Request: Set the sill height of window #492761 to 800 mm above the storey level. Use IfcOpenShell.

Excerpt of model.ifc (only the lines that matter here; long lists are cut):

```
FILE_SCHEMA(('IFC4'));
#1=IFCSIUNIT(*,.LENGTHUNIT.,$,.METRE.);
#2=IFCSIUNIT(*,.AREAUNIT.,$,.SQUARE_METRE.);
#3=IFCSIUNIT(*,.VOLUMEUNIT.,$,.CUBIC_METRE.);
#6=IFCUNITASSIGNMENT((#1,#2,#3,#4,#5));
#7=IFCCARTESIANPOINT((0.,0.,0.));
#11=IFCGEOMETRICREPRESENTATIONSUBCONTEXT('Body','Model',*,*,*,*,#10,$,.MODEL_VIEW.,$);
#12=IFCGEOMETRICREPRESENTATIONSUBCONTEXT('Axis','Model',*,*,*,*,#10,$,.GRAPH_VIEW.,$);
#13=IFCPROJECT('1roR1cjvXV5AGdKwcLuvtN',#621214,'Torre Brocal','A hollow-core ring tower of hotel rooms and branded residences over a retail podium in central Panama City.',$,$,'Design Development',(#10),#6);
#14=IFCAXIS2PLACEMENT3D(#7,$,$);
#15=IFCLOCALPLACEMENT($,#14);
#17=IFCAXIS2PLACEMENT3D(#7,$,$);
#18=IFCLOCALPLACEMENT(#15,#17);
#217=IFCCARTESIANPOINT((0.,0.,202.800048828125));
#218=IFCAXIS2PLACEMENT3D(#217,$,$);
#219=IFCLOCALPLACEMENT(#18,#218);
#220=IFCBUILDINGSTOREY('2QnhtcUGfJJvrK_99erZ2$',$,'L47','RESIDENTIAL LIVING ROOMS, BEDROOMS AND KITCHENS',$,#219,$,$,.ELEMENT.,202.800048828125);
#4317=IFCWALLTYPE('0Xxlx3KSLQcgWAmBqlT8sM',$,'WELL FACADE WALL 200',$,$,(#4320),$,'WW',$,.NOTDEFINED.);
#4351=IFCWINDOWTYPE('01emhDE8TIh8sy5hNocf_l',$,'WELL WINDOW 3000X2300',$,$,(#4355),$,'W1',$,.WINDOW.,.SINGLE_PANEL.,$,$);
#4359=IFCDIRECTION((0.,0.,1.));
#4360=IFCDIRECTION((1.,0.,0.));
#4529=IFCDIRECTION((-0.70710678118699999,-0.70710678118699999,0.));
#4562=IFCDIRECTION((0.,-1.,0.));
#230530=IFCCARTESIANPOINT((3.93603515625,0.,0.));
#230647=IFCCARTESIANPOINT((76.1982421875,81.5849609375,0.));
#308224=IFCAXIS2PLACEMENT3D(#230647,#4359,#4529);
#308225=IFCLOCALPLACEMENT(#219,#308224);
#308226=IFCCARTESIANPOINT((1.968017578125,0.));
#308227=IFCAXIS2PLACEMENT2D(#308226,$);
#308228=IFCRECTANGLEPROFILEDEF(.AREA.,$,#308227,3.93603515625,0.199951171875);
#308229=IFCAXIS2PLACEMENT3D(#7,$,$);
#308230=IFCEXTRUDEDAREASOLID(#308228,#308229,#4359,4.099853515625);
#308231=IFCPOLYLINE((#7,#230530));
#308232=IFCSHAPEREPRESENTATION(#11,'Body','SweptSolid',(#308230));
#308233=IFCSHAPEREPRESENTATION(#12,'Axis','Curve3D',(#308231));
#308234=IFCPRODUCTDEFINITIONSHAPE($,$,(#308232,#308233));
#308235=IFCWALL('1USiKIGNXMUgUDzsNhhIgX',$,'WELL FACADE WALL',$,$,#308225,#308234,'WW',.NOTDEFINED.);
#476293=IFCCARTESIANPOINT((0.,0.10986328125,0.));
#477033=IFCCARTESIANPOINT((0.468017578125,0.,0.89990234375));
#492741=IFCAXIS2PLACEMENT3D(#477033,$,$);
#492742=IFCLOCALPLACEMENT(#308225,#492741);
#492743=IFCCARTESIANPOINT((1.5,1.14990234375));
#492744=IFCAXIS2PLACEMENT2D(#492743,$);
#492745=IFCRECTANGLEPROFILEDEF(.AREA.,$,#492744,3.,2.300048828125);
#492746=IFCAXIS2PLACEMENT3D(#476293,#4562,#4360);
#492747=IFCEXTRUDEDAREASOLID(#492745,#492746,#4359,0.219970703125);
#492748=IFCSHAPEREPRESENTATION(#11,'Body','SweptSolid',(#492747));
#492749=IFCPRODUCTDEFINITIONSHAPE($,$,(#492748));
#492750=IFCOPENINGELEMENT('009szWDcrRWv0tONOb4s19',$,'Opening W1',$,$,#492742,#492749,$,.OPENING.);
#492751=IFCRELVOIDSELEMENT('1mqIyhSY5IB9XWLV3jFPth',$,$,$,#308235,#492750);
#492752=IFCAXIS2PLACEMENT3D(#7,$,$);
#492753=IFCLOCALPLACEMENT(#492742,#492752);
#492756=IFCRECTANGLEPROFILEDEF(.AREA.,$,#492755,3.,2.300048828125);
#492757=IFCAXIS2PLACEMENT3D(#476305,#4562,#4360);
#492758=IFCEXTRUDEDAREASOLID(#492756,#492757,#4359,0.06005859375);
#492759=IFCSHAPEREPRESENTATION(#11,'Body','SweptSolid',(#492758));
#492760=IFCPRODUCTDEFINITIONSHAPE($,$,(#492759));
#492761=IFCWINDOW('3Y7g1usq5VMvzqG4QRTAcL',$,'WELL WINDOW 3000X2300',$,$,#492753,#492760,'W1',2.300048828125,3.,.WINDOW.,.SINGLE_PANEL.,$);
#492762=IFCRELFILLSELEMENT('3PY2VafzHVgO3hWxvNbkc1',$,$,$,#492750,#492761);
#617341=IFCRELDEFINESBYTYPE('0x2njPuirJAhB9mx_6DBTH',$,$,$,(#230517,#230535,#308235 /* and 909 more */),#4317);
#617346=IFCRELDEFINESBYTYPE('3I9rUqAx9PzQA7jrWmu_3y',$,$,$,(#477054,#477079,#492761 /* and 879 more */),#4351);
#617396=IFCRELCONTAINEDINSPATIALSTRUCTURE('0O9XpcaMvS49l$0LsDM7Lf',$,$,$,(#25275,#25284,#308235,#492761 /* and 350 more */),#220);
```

```python
import numpy as np
import ifcopenshell
import ifcopenshell.api.geometry
import ifcopenshell.geom
import ifcopenshell.util.element
import ifcopenshell.util.placement
import ifcopenshell.util.shape
import ifcopenshell.util.unit

model = ifcopenshell.open("model.ifc")
unit_scale = ifcopenshell.util.unit.calculate_unit_scale(model)

window = model.by_guid("3Y7g1usq5VMvzqG4QRTAcL")
opening = window.FillsVoids[0].RelatingOpeningElement
storey = ifcopenshell.util.element.get_container(window, ifc_class="IfcBuildingStorey")
level = ifcopenshell.util.placement.get_local_placement(storey.ObjectPlacement)[2, 3]

# The opening's origin need not be at the sill, so measure its lowest point.
shape = ifcopenshell.geom.create_shape(ifcopenshell.geom.settings(), opening)
bottom = ifcopenshell.util.shape.get_shape_bottom_elevation(shape, shape.geometry) / unit_scale
dz = level + 0.8 - bottom

shift = np.array([0.0, 0.0, dz])
# The window is placed relative to its opening, so it follows when the opening moves.
matrix = ifcopenshell.util.placement.get_local_placement(opening.ObjectPlacement)
matrix[:3, 3] += shift
ifcopenshell.api.geometry.edit_object_placement(
    model, product=opening, matrix=matrix, is_si=False, should_transform_children=True
)

print(f"moved by {dz * unit_scale:+.3f} m")

model.write("model_rev.ifc")
```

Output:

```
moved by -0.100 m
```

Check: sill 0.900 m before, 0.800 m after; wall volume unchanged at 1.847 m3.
